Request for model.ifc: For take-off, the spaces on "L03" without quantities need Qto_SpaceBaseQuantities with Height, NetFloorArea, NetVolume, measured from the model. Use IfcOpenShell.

First a look at what the model holds.

```python
import ifcopenshell
import ifcopenshell.util.element
import ifcopenshell.util.unit

model = ifcopenshell.open("model.ifc")
print(model.schema)
for unit_type in ("LENGTHUNIT", "AREAUNIT", "VOLUMEUNIT"):
    print(unit_type, ifcopenshell.util.unit.calculate_unit_scale(model, unit_type))
storey = next(s for s in model.by_type("IfcBuildingStorey") if s.Name == "L03")
spaces = [e for e in ifcopenshell.util.element.get_decomposition(storey) if e.is_a("IfcSpace")]
for e in sorted(spaces, key=lambda e: e.id()):
    print(e.id(), e.is_a(), e.Name, list(ifcopenshell.util.element.get_psets(e, qtos_only=True)), sep=" | ")
```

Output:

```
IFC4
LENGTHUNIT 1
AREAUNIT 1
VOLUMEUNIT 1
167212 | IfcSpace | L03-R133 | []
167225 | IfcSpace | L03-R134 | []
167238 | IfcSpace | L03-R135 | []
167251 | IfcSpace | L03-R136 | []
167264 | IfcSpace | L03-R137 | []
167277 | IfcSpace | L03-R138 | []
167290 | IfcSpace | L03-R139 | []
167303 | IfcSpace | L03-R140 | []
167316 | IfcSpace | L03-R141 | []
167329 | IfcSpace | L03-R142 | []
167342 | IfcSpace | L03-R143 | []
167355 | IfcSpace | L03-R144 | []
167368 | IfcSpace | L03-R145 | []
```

```python
import ifcopenshell
import ifcopenshell.api.pset
import ifcopenshell.geom
import ifcopenshell.util.element
import ifcopenshell.util.shape
import ifcopenshell.util.unit

model = ifcopenshell.open("model.ifc")
unit_scale = ifcopenshell.util.unit.calculate_unit_scale(model)
area_scale = ifcopenshell.util.unit.calculate_unit_scale(model, "AREAUNIT")
volume_scale = ifcopenshell.util.unit.calculate_unit_scale(model, "VOLUMEUNIT")
settings = ifcopenshell.geom.settings()

storey = next(s for s in model.by_type("IfcBuildingStorey") if s.Name == "L03")
spaces = [e for e in ifcopenshell.util.element.get_decomposition(storey) if e.is_a("IfcSpace")]

for e in sorted(spaces, key=lambda e: e.id()):
    if ifcopenshell.util.element.get_psets(e, qtos_only=True, should_inherit=False):
        continue
    # Geometry comes back in metres, in the element's own axes.
    shape = ifcopenshell.geom.create_shape(settings, e)
    values = {
        "Height": ifcopenshell.util.shape.get_z(shape.geometry) / unit_scale,
        "NetFloorArea": ifcopenshell.util.shape.get_footprint_area(shape.geometry) / area_scale,
        "NetVolume": ifcopenshell.util.shape.get_volume(shape.geometry) / volume_scale,
    }
    qto = ifcopenshell.api.pset.add_qto(model, product=e, name="Qto_SpaceBaseQuantities")
    ifcopenshell.api.pset.edit_qto(model, qto=qto, properties=values)
    print(e.id(), {k: round(v, 3) for k, v in values.items()})

model.write("model_edited.ifc")
```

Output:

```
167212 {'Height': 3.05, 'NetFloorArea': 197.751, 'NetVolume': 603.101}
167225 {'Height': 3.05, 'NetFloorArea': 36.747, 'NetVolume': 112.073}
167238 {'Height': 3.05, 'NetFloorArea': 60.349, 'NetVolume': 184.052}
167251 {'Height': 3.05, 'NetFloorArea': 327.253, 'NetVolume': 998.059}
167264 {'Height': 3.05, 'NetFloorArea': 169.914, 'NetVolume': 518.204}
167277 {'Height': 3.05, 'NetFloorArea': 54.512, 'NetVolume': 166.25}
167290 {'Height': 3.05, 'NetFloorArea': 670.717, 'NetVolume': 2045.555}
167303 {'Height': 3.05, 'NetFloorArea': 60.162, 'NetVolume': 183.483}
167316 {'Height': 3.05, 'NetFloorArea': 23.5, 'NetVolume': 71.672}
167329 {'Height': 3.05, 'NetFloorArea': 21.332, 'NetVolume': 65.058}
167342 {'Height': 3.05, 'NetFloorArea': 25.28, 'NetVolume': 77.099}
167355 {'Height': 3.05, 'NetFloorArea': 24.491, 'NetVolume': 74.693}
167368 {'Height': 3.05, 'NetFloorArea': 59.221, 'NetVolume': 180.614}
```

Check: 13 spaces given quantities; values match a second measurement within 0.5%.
